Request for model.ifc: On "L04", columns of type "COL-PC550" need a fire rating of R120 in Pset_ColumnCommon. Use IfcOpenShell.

First a look at what the model holds.

```python
import ifcopenshell
import ifcopenshell.util.element

model = ifcopenshell.open("model.ifc")
print(model.schema)
storey = next(s for s in model.by_type("IfcBuildingStorey") if s.Name == "L04")
columns = [e for e in ifcopenshell.util.element.get_decomposition(storey) if e.is_a("IfcColumn")]
seen = {}
for e in columns:
    element_type = ifcopenshell.util.element.get_type(e)
    key = (element_type.Name if element_type != e and element_type else None, ifcopenshell.util.element.get_pset(e, "Pset_ColumnCommon", "FireRating"))
    seen[key] = seen.get(key, 0) + 1
for (name, value), count in sorted(seen.items(), key=str):
    print(count, "x", name, "|", value)
```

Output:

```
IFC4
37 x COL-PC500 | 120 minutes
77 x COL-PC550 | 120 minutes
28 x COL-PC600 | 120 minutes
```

```python
import ifcopenshell
import ifcopenshell.api.pset
import ifcopenshell.util.element

model = ifcopenshell.open("model.ifc")

storey = next(s for s in model.by_type("IfcBuildingStorey") if s.Name == "L04")
columns = [e for e in ifcopenshell.util.element.get_decomposition(storey) if e.is_a("IfcColumn")]

count = 0
for e in columns:
    element_type = ifcopenshell.util.element.get_type(e)
    if element_type in (None, e) or element_type.Name != "COL-PC550":
        continue
    # add_pset returns the element's existing set when there is one.
    pset = ifcopenshell.api.pset.add_pset(model, product=e, name="Pset_ColumnCommon")
    ifcopenshell.api.pset.edit_pset(model, pset=pset, properties={"FireRating": "R120"})
    count += 1

print(count, "columns updated")

model.write("model-out.ifc")
```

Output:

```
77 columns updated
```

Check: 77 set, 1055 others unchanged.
